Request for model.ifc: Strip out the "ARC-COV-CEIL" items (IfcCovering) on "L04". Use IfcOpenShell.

First a look at what the model holds.

```python
import ifcopenshell
import ifcopenshell.util.element

model = ifcopenshell.open("model.ifc")
print(model.schema)
storey = next(s for s in model.by_type("IfcBuildingStorey") if s.Name == "L04")
coverings = [e for e in ifcopenshell.util.element.get_decomposition(storey) if e.is_a("IfcCovering")]
seen = {}
for e in coverings:
    element_type = ifcopenshell.util.element.get_type(e)
    name = element_type.Name if element_type not in (None, e) else None
    seen[name] = seen.get(name, 0) + 1
for name, count in sorted(seen.items(), key=str):
    print(count, "x", name)
```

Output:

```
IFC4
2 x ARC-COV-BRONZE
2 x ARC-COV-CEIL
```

```python
import ifcopenshell
import ifcopenshell.api.root
import ifcopenshell.util.element

model = ifcopenshell.open("model.ifc")

storey = next(s for s in model.by_type("IfcBuildingStorey") if s.Name == "L04")
coverings = [e for e in ifcopenshell.util.element.get_decomposition(storey) if e.is_a("IfcCovering")]
targets = [e for e in coverings if (t := ifcopenshell.util.element.get_type(e)) not in (None, e) and t.Name == "ARC-COV-CEIL"]

for e in targets:
    ifcopenshell.api.root.remove_product(model, product=e)
print(len(targets), "removed")

model.write("model-out.ifc")
```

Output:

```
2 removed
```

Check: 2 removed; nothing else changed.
